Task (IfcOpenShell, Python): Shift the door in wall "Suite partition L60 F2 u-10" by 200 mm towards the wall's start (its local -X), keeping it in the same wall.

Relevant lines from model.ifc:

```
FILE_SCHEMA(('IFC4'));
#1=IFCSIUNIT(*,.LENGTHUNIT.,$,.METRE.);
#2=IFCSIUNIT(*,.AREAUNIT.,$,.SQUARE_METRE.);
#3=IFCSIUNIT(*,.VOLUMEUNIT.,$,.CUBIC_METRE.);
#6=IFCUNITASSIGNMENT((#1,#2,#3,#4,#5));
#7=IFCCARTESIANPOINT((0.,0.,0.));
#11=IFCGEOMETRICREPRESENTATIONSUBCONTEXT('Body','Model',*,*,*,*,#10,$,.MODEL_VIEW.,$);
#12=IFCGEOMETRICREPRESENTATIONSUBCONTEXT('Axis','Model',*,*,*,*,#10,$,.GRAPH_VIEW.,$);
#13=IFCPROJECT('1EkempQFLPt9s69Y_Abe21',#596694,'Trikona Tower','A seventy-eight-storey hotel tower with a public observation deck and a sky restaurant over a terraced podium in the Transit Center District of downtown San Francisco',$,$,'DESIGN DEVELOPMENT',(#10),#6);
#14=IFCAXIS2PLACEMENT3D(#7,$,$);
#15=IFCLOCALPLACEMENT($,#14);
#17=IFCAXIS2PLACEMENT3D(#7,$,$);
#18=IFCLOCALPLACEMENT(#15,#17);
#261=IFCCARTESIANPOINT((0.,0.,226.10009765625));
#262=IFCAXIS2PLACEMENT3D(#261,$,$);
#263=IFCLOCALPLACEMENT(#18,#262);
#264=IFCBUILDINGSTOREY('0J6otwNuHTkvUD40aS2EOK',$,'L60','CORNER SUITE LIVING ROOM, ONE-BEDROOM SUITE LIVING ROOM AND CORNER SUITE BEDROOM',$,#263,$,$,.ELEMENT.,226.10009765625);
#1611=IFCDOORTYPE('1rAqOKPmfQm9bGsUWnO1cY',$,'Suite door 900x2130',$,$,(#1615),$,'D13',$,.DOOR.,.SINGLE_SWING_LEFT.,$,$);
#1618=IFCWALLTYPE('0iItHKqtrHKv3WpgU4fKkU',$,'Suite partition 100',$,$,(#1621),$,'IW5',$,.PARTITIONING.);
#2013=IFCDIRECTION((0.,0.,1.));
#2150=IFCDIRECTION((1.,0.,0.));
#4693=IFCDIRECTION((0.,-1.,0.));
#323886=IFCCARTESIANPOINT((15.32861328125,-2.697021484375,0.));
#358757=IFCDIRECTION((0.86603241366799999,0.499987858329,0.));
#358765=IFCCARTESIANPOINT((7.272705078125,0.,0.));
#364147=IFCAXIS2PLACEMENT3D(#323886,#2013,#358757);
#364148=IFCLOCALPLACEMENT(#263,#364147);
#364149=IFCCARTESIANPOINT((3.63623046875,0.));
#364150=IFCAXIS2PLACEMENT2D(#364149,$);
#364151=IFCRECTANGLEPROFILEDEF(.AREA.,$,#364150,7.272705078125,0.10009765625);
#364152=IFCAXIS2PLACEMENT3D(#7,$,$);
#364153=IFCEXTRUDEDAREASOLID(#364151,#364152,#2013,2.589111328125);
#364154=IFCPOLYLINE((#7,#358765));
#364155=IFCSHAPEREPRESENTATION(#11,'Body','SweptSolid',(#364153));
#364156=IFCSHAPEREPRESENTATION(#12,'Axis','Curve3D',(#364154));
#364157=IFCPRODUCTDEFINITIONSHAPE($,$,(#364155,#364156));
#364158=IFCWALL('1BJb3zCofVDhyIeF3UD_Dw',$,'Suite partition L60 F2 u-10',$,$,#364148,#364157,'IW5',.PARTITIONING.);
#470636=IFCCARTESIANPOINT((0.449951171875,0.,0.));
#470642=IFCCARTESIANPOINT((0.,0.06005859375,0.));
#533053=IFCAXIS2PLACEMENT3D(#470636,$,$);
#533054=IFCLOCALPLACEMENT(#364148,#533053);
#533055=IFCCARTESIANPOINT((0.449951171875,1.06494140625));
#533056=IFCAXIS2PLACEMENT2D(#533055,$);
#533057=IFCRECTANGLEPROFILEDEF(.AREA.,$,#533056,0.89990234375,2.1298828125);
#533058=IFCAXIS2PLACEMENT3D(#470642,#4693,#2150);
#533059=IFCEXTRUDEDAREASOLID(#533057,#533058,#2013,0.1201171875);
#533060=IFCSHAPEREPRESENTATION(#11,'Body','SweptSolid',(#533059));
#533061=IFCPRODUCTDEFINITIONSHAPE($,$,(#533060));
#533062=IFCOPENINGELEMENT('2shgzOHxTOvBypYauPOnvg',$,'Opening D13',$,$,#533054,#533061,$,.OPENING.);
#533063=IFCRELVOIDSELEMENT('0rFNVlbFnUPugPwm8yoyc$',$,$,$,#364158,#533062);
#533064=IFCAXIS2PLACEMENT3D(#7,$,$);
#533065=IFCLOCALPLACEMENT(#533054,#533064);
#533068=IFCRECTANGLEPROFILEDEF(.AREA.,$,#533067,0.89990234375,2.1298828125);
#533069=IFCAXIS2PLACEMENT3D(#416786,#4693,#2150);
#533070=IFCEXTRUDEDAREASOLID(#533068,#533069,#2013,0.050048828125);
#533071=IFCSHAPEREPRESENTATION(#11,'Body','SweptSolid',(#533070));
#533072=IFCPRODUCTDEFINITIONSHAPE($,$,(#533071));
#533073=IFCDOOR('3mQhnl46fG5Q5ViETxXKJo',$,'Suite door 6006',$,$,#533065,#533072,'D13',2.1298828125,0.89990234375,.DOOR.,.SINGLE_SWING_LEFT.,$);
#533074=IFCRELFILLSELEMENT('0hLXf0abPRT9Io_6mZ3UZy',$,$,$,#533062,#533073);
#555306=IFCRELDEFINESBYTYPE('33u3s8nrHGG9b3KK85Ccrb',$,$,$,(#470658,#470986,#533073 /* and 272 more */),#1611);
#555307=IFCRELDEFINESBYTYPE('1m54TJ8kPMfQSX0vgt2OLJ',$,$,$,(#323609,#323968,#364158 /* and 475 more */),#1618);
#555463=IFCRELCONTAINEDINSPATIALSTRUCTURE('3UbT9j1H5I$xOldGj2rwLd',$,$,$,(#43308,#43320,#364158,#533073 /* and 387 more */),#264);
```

```python
import ifcopenshell
import ifcopenshell.api.geometry
import ifcopenshell.util.placement
import ifcopenshell.util.unit

model = ifcopenshell.open("model.ifc")
unit_scale = ifcopenshell.util.unit.calculate_unit_scale(model)

door = model.by_guid("3mQhnl46fG5Q5ViETxXKJo")
opening = door.FillsVoids[0].RelatingOpeningElement
wall = opening.VoidsElements[0].RelatingBuildingElement

wall_matrix = ifcopenshell.util.placement.get_local_placement(wall.ObjectPlacement)
shift = wall_matrix[:3, 0] * -0.2 / unit_scale
before = ifcopenshell.util.placement.get_local_placement(door.ObjectPlacement)[:3, 3].copy()

# The door is placed relative to its opening, so it follows when the opening moves.
matrix = ifcopenshell.util.placement.get_local_placement(opening.ObjectPlacement)
matrix[:3, 3] += shift
ifcopenshell.api.geometry.edit_object_placement(
    model, product=opening, matrix=matrix, is_si=False, should_transform_children=True
)

after = ifcopenshell.util.placement.get_local_placement(door.ObjectPlacement)[:3, 3]
print("door moved by", (after - before).round(3) + 0.0)

model.write("model_updated.ifc")
```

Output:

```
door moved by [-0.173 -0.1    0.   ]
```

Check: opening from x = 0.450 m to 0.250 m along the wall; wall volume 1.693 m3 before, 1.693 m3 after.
